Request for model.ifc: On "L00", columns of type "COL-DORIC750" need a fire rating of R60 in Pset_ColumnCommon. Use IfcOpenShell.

First a look at what the model holds.

```python
import ifcopenshell
import ifcopenshell.util.element

model = ifcopenshell.open("model.ifc")
print(model.schema)
storey = next(s for s in model.by_type("IfcBuildingStorey") if s.Name == "L00")
columns = [e for e in ifcopenshell.util.element.get_decomposition(storey) if e.is_a("IfcColumn")]
seen = {}
for e in columns:
    element_type = ifcopenshell.util.element.get_type(e)
    key = (element_type.Name if element_type != e and element_type else None, ifcopenshell.util.element.get_pset(e, "Pset_ColumnCommon", "FireRating"))
    seen[key] = seen.get(key, 0) + 1
for (name, value), count in sorted(seen.items(), key=str):
    print(count, "x", name, "|", value)
```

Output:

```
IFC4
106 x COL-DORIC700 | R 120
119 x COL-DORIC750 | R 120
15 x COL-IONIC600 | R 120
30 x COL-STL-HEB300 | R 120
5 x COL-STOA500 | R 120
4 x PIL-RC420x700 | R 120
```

```python
import ifcopenshell
import ifcopenshell.api.pset
import ifcopenshell.util.element

model = ifcopenshell.open("model.ifc")

storey = next(s for s in model.by_type("IfcBuildingStorey") if s.Name == "L00")
columns = [e for e in ifcopenshell.util.element.get_decomposition(storey) if e.is_a("IfcColumn")]

count = 0
for e in columns:
    element_type = ifcopenshell.util.element.get_type(e)
    if element_type in (None, e) or element_type.Name != "COL-DORIC750":
        continue
    # add_pset returns the element's existing set when there is one.
    pset = ifcopenshell.api.pset.add_pset(model, product=e, name="Pset_ColumnCommon")
    ifcopenshell.api.pset.edit_pset(model, pset=pset, properties={"FireRating": "R60"})
    count += 1

print(count, "columns updated")

model.write("model_updated.ifc")
```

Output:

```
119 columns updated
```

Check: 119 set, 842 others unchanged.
